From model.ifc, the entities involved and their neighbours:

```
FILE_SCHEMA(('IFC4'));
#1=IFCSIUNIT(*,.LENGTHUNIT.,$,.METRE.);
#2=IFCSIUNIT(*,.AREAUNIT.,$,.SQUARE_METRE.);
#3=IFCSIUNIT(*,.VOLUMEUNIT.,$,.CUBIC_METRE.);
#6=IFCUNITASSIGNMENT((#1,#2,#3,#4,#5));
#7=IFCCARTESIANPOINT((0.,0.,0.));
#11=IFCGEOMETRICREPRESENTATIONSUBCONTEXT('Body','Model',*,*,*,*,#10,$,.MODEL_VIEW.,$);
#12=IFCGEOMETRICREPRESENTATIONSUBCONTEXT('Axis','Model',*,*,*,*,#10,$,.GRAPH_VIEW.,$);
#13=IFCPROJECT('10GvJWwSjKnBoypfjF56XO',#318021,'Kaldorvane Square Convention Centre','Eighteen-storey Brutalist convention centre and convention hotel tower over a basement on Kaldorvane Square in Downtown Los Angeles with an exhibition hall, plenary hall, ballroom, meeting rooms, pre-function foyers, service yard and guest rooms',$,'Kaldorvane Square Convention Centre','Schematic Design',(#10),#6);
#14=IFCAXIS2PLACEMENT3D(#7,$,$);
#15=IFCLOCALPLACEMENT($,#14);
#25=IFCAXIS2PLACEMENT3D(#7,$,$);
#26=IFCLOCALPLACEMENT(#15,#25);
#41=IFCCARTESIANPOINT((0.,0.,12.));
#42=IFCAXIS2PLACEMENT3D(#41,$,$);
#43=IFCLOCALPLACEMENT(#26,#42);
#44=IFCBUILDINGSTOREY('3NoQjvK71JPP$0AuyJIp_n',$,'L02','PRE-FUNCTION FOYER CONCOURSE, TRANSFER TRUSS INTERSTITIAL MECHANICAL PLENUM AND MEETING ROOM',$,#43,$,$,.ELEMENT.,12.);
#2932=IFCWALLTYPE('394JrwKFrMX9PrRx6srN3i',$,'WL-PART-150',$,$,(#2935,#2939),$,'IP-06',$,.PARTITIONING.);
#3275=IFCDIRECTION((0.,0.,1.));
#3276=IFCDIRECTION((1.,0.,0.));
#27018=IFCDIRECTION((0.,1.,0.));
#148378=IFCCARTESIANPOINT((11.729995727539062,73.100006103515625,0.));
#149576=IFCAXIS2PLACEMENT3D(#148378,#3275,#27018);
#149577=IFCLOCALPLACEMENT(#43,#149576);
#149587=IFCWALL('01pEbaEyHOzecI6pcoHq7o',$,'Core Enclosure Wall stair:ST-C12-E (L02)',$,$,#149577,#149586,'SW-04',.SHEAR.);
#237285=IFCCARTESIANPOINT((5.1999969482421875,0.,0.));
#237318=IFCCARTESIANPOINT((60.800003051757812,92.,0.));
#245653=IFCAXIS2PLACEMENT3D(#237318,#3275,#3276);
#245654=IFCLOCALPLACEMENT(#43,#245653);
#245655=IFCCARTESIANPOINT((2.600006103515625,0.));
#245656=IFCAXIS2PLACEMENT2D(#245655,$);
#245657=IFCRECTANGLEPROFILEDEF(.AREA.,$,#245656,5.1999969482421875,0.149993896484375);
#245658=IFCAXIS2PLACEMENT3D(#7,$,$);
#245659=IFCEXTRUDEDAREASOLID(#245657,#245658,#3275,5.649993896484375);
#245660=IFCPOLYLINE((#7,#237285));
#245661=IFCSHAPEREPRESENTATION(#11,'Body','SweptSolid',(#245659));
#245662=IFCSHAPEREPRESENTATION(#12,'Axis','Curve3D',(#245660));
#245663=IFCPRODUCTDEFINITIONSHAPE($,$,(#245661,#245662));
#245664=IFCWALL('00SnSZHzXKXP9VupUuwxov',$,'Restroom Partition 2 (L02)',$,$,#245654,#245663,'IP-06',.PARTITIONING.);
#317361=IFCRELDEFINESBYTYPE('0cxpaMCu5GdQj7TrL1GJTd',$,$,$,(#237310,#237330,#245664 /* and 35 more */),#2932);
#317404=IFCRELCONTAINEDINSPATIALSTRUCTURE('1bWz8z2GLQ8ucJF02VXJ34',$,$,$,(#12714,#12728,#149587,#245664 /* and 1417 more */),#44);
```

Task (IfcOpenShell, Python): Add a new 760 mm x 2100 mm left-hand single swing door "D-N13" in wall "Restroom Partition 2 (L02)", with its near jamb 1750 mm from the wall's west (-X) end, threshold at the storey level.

```python
import numpy as np
import ifcopenshell
import ifcopenshell.api.feature
import ifcopenshell.api.geometry
import ifcopenshell.api.root
import ifcopenshell.api.spatial
import ifcopenshell.geom
import ifcopenshell.util.element
import ifcopenshell.util.placement
import ifcopenshell.util.representation
import ifcopenshell.util.shape
import ifcopenshell.util.unit

model = ifcopenshell.open("model.ifc")
unit_scale = ifcopenshell.util.unit.calculate_unit_scale(model)
settings = ifcopenshell.geom.settings()


def volume(element):
    """Net volume in cubic metres, openings subtracted."""
    shape = ifcopenshell.geom.create_shape(settings, element)
    return ifcopenshell.util.shape.get_volume(shape.geometry)


wall = model.by_guid("00SnSZHzXKXP9VupUuwxov")
storey = ifcopenshell.util.element.get_container(wall, ifc_class="IfcBuildingStorey")
context = ifcopenshell.util.representation.get_context(model, "Model", "Body", "MODEL_VIEW")
before = volume(wall)

width, height, from_end, sill = 0.76, 2.1, 1.75, 0.0  # metres

# The wall runs along its own X axis, and the end named is its -X end.
wall_shape = ifcopenshell.geom.create_shape(settings, wall)
x, y, z = ifcopenshell.util.shape.get_vertices(wall_shape.geometry).T
start = x.min() + from_end
face, thickness = float(y.min()), float(y.max() - y.min())
wall_matrix = ifcopenshell.util.placement.get_local_placement(wall.ObjectPlacement)
level = ifcopenshell.util.placement.get_local_placement(storey.ObjectPlacement)[2, 3]


def in_wall(x, y):
    """Placement at x, y metres in the wall's axes, at sill height."""
    matrix = wall_matrix.copy()
    matrix[:, 3] = wall_matrix @ np.array([x / unit_scale, y / unit_scale, 0.0, 1.0])
    matrix[2, 3] = level + sill / unit_scale
    return matrix


# Opening: a box that overshoots both wall faces by 50 mm.
opening = ifcopenshell.api.root.create_entity(model, ifc_class="IfcOpeningElement", predefined_type="OPENING")
box = ifcopenshell.api.geometry.add_wall_representation(
    model, context=context, length=width, height=height, thickness=thickness + 0.1
)
ifcopenshell.api.geometry.assign_representation(model, product=opening, representation=box)
ifcopenshell.api.geometry.edit_object_placement(model, product=opening, matrix=in_wall(start, face - 0.05), is_si=False)
ifcopenshell.api.feature.add_feature(model, feature=opening, element=wall)

door = ifcopenshell.api.root.create_entity(model, ifc_class="IfcDoor", name="D-N13", predefined_type="DOOR")
door.OverallWidth, door.OverallHeight = width / unit_scale, height / unit_scale
door.OperationType = "SINGLE_SWING_LEFT"
body = ifcopenshell.api.geometry.add_door_representation(
    model,
    context=context,
    overall_width=door.OverallWidth,
    overall_height=door.OverallHeight,
    operation_type="SINGLE_SWING_LEFT",
    lining_properties={"LiningDepth": thickness / unit_scale, "ThresholdDepth": thickness / unit_scale},
)
ifcopenshell.api.geometry.assign_representation(model, product=door, representation=body)
ifcopenshell.api.spatial.assign_container(model, products=[door], relating_structure=storey)
ifcopenshell.api.feature.add_filling(model, opening=opening, element=door)

# The lining spans the wall, so the door starts at the wall face.
ifcopenshell.api.geometry.edit_object_placement(model, product=door, matrix=in_wall(start, face), is_si=False)

after = volume(wall)

print(f"wall volume {before:.3f} -> {after:.3f} m3")

model.write("model_edited.ifc")
```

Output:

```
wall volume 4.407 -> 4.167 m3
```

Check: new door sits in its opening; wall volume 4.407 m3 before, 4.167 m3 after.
